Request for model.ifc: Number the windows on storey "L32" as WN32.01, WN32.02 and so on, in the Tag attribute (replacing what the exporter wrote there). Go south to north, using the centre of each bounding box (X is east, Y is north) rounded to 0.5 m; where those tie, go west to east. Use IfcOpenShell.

First a look at what the model holds.

```python
import ifcopenshell
import ifcopenshell.util.element
import ifcopenshell.util.placement

model = ifcopenshell.open("model.ifc")
print(model.schema)
storey = next(s for s in model.by_type("IfcBuildingStorey") if s.Name == "L32")
windows = [e for e in ifcopenshell.util.element.get_decomposition(storey) if e.is_a("IfcWindow")]
for e in sorted(windows, key=lambda e: e.id()):
    origin = ifcopenshell.util.placement.get_local_placement(e.ObjectPlacement)[:3, 3]
    print(e.id(), e.Tag, e.Name, origin.round(2) + 0.0, sep=" | ")
```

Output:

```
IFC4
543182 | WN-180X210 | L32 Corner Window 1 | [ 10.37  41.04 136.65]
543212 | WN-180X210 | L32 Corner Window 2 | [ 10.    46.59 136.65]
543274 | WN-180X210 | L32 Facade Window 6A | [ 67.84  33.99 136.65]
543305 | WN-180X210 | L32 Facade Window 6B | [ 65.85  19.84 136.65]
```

```python
import ifcopenshell
import ifcopenshell.geom
import ifcopenshell.util.element
import ifcopenshell.util.shape

model = ifcopenshell.open("model.ifc")
settings = ifcopenshell.geom.settings()
settings.set("use-world-coords", True)


def centre(element):
    shape = ifcopenshell.geom.create_shape(settings, element)
    return ifcopenshell.util.shape.get_bbox_centroid(shape.geometry)


storey = next(s for s in model.by_type("IfcBuildingStorey") if s.Name == "L32")
windows = [e for e in ifcopenshell.util.element.get_decomposition(storey) if e.is_a("IfcWindow")]

# Insertion points can sit at a corner or the storey origin, so sort by the geometry (in metres).
centres = {e: centre(e) for e in windows}
windows.sort(key=lambda e: (round(centres[e][1] / 0.5), centres[e][0]))

for i, e in enumerate(windows, start=1):
    number = f"WN32.{i:02d}"
    e.Tag = number
    print(e.id(), number)

model.write("model_edited.ifc")
```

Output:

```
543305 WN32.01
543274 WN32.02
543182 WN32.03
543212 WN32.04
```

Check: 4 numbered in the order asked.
